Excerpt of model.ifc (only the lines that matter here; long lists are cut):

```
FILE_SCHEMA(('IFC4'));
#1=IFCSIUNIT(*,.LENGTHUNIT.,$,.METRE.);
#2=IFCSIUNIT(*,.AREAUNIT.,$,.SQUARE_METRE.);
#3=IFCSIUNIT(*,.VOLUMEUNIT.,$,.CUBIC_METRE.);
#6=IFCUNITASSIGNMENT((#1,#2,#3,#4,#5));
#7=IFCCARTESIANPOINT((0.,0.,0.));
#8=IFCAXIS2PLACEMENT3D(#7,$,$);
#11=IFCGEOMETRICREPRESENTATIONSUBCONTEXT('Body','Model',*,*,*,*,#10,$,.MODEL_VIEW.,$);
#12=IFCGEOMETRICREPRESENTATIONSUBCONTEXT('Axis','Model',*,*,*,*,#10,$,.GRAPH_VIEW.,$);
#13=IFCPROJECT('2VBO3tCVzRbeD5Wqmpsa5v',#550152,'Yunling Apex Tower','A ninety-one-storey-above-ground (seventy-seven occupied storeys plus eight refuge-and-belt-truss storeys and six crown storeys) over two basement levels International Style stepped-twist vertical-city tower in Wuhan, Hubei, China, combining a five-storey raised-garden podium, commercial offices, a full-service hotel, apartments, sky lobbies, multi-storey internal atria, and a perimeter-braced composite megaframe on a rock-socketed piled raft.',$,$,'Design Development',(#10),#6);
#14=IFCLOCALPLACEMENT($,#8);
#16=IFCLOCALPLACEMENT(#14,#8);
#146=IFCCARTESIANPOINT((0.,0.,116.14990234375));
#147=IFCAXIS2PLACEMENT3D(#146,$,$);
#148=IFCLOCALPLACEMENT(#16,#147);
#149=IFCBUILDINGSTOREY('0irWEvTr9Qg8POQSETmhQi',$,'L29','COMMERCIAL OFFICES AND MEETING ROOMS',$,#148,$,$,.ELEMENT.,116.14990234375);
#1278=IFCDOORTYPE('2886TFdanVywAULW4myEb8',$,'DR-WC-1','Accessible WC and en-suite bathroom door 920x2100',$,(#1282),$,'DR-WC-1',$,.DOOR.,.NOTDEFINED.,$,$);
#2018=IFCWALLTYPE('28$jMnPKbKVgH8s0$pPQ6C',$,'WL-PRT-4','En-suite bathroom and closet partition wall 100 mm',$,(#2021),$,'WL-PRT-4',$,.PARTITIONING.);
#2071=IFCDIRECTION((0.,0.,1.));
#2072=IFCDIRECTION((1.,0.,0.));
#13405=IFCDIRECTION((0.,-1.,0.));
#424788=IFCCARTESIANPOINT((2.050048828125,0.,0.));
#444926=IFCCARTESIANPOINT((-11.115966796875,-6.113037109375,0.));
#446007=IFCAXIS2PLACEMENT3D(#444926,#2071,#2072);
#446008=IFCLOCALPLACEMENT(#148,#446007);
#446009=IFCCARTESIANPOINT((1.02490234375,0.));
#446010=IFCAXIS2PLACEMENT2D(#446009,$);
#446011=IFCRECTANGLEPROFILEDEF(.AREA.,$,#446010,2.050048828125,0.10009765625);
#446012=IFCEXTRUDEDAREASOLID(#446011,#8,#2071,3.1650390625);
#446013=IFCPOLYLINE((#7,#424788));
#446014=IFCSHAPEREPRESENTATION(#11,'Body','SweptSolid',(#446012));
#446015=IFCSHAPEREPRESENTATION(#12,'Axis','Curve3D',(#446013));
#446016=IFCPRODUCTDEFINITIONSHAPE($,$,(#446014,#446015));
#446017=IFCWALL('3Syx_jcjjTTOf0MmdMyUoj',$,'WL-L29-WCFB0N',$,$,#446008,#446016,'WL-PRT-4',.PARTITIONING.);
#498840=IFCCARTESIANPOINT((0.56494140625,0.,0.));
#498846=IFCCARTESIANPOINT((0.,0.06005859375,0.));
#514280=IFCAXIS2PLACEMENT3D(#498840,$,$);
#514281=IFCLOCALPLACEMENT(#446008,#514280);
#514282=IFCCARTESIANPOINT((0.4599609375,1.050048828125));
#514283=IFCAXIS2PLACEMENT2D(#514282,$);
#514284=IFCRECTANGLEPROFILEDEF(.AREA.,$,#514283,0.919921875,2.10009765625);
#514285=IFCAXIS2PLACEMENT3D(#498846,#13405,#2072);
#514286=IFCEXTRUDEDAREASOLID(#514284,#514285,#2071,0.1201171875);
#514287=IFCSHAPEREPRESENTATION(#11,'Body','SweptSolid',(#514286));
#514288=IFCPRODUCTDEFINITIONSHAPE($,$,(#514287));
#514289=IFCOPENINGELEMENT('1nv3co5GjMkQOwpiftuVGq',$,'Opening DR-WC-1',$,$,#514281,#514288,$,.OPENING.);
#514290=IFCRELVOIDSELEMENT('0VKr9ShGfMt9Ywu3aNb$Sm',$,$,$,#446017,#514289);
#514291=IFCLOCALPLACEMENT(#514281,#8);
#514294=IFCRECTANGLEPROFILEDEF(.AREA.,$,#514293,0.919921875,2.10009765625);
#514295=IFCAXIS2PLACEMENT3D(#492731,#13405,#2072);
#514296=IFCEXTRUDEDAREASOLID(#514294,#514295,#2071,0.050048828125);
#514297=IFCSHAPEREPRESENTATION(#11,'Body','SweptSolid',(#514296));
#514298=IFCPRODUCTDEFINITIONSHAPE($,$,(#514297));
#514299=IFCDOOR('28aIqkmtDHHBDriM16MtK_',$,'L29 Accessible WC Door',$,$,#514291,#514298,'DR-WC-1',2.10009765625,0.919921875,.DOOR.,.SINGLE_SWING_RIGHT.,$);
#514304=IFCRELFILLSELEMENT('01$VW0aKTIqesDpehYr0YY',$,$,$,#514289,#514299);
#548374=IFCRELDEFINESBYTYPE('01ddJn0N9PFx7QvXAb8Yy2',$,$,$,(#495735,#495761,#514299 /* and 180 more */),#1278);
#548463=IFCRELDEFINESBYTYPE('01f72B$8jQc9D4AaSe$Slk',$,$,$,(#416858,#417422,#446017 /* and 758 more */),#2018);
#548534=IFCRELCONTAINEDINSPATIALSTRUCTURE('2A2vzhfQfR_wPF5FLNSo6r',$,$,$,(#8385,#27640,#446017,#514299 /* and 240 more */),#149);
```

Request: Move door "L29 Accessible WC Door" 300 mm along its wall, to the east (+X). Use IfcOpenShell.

```python
import ifcopenshell
import ifcopenshell.api.geometry
import ifcopenshell.util.placement
import ifcopenshell.util.unit

model = ifcopenshell.open("model.ifc")
unit_scale = ifcopenshell.util.unit.calculate_unit_scale(model)

door = model.by_guid("28aIqkmtDHHBDriM16MtK_")
opening = door.FillsVoids[0].RelatingOpeningElement
wall = opening.VoidsElements[0].RelatingBuildingElement

wall_matrix = ifcopenshell.util.placement.get_local_placement(wall.ObjectPlacement)
shift = wall_matrix[:3, 0] * 0.3 / unit_scale
before = ifcopenshell.util.placement.get_local_placement(door.ObjectPlacement)[:3, 3].copy()

# The door is placed relative to its opening, so it follows when the opening moves.
matrix = ifcopenshell.util.placement.get_local_placement(opening.ObjectPlacement)
matrix[:3, 3] += shift
ifcopenshell.api.geometry.edit_object_placement(
    model, product=opening, matrix=matrix, is_si=False, should_transform_children=True
)

after = ifcopenshell.util.placement.get_local_placement(door.ObjectPlacement)[:3, 3]
print("door moved by", (after - before).round(3) + 0.0)

model.write("model_updated.ifc")
```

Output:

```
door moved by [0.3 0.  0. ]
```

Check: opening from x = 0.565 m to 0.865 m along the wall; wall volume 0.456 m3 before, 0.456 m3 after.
